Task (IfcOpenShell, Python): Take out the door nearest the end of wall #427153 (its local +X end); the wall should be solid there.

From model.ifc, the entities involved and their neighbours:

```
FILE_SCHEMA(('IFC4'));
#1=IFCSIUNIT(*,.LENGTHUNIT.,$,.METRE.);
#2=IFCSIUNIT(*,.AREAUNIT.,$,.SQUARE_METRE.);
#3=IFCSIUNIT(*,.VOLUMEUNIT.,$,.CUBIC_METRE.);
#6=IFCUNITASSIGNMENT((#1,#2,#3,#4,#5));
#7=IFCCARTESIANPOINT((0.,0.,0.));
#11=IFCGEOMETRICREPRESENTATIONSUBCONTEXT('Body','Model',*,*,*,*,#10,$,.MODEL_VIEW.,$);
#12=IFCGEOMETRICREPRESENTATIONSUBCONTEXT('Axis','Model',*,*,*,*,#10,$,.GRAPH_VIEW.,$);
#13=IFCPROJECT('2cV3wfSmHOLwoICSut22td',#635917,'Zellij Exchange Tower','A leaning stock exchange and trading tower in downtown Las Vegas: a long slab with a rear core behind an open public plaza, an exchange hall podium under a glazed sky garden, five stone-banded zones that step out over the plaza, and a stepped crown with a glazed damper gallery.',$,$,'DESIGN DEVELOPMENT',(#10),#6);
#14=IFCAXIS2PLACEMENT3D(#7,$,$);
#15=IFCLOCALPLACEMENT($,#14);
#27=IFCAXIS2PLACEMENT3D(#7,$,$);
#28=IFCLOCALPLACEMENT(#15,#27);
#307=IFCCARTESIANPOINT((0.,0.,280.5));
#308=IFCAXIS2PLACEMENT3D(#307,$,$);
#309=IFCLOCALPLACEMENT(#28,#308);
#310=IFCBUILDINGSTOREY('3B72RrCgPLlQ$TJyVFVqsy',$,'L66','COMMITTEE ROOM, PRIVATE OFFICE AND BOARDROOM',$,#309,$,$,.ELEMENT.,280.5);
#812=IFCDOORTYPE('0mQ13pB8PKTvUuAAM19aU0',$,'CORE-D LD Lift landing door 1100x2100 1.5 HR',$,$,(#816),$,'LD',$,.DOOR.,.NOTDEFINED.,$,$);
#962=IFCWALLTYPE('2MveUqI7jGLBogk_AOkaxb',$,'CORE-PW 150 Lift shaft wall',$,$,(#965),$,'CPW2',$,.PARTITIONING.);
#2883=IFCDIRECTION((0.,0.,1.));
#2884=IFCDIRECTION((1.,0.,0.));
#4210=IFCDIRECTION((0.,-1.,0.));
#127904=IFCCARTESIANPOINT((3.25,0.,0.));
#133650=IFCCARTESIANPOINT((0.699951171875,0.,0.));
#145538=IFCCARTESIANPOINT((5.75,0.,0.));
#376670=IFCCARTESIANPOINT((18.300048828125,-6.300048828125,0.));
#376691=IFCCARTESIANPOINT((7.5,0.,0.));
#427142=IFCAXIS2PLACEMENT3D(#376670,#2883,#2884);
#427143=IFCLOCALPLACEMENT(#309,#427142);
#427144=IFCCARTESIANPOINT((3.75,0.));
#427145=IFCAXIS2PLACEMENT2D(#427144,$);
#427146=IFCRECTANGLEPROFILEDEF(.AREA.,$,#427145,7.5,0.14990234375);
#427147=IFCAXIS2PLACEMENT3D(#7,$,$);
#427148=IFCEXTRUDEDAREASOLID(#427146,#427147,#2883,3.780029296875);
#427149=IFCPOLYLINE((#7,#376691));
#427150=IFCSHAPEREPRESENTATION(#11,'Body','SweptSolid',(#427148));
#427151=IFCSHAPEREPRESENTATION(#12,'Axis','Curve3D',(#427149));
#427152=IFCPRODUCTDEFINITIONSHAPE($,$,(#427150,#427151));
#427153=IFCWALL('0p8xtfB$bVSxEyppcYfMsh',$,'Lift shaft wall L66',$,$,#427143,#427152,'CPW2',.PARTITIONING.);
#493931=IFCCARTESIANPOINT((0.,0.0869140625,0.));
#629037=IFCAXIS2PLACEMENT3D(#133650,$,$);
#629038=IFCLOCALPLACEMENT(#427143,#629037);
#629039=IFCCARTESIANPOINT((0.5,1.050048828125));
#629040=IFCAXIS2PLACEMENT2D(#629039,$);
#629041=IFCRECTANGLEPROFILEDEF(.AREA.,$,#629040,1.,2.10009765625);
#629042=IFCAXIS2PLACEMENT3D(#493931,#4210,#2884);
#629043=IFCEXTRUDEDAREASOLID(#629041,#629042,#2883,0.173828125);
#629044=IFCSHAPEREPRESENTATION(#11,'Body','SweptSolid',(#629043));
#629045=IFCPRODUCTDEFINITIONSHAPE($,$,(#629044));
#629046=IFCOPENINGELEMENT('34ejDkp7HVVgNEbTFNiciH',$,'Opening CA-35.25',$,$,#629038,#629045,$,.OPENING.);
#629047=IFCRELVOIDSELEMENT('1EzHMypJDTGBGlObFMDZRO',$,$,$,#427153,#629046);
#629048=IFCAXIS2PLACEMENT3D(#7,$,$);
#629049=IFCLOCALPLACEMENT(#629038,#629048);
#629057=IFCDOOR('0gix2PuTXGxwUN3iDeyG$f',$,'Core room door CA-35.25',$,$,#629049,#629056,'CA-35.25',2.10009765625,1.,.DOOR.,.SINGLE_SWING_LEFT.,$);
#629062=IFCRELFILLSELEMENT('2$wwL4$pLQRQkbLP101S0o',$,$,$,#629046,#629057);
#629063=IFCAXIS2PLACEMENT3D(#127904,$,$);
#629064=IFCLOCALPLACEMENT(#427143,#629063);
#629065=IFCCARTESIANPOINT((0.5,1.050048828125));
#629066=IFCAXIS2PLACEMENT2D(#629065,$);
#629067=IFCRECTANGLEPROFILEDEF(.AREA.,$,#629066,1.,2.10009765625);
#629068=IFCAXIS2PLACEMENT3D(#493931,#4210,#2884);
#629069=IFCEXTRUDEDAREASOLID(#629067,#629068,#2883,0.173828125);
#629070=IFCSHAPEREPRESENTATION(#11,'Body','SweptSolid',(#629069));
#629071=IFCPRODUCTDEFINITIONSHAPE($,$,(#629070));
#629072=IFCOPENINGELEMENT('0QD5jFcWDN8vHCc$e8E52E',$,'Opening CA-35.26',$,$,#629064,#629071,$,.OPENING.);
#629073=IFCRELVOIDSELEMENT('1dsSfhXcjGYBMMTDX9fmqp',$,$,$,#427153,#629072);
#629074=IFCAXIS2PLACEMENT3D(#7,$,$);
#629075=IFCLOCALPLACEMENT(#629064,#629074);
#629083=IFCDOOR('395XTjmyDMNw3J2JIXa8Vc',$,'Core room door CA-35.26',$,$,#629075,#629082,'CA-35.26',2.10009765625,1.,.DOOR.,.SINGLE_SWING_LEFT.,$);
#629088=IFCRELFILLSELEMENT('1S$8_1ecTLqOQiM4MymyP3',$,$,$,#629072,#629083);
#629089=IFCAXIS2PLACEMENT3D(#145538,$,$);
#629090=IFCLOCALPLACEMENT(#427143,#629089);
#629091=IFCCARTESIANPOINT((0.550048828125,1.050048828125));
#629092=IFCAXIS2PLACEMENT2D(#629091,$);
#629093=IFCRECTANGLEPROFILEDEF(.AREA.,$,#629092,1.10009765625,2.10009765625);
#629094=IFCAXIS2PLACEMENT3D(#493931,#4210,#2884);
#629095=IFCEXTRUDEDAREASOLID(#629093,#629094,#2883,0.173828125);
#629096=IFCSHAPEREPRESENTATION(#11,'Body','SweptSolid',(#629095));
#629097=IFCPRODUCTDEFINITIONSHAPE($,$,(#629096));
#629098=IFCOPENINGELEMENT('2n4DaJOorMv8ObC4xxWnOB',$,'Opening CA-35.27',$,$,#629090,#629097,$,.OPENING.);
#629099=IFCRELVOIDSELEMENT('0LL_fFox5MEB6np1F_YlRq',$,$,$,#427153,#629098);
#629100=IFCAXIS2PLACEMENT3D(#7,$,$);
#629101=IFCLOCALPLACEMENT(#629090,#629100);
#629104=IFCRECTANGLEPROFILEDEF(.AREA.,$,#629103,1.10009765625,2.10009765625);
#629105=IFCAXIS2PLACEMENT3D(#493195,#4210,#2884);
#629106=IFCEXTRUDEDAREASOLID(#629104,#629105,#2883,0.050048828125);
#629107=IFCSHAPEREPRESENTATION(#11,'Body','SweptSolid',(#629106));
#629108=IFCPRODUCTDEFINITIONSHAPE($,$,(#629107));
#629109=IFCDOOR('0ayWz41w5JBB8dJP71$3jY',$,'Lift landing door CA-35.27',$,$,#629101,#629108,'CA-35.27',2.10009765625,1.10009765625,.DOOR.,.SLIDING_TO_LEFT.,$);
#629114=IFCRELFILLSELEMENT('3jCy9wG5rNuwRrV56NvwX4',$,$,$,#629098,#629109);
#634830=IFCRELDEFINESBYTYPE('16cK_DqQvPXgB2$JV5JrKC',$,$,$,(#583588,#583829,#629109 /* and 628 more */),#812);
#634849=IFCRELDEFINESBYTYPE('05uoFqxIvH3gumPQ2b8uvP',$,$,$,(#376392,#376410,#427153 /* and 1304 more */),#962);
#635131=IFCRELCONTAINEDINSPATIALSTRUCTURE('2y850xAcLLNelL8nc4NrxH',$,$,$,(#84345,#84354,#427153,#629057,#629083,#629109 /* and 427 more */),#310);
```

```python
import ifcopenshell
import ifcopenshell.api.feature
import ifcopenshell.api.root
import ifcopenshell.geom
import ifcopenshell.util.shape

model = ifcopenshell.open("model.ifc")
settings = ifcopenshell.geom.settings()


def volume(element):
    """Net volume in cubic metres, openings subtracted."""
    shape = ifcopenshell.geom.create_shape(settings, element)
    return ifcopenshell.util.shape.get_volume(shape.geometry)


door = model.by_guid("0ayWz41w5JBB8dJP71$3jY")
opening = door.FillsVoids[0].RelatingOpeningElement
wall = opening.VoidsElements[0].RelatingBuildingElement
before = volume(wall)

ifcopenshell.api.root.remove_product(model, product=door)
ifcopenshell.api.feature.remove_feature(model, feature=opening)

after = volume(wall)

print(f"wall volume {before:.3f} -> {after:.3f} m3")

model.write("model_rev.ifc")
```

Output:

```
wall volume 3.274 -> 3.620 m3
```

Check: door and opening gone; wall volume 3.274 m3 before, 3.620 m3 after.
